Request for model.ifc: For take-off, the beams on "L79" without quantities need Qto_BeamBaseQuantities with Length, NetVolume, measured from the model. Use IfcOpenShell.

First a look at what the model holds.

```python
import ifcopenshell
import ifcopenshell.util.element
import ifcopenshell.util.unit

model = ifcopenshell.open("model.ifc")
print(model.schema)
for unit_type in ("LENGTHUNIT", "AREAUNIT", "VOLUMEUNIT"):
    print(unit_type, ifcopenshell.util.unit.calculate_unit_scale(model, unit_type))
storey = next(s for s in model.by_type("IfcBuildingStorey") if s.Name == "L79")
beams = [e for e in ifcopenshell.util.element.get_decomposition(storey) if e.is_a("IfcBeam")]
for e in sorted(beams, key=lambda e: e.id()):
    print(e.id(), e.is_a(), e.Name, list(ifcopenshell.util.element.get_psets(e, qtos_only=True)), sep=" | ")
```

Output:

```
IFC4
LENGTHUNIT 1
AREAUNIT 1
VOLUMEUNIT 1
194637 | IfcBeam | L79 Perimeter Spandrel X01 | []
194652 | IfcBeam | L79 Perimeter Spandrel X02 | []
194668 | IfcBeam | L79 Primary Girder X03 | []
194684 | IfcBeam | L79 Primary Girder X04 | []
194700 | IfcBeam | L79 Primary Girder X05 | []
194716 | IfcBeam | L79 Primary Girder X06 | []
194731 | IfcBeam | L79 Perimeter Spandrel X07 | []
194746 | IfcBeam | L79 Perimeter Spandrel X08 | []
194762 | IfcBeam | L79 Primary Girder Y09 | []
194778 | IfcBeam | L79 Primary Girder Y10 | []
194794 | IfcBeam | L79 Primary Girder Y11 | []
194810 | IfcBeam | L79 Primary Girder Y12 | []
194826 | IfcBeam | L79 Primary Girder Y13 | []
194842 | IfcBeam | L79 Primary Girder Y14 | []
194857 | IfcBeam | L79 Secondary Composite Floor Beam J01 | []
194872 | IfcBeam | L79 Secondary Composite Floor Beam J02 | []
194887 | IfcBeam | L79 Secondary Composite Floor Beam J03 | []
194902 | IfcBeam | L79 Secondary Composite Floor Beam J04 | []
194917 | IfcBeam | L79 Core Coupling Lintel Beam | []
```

```python
import ifcopenshell
import ifcopenshell.api.pset
import ifcopenshell.geom
import ifcopenshell.util.element
import ifcopenshell.util.shape
import ifcopenshell.util.unit

model = ifcopenshell.open("model.ifc")
unit_scale = ifcopenshell.util.unit.calculate_unit_scale(model)
volume_scale = ifcopenshell.util.unit.calculate_unit_scale(model, "VOLUMEUNIT")
settings = ifcopenshell.geom.settings()

storey = next(s for s in model.by_type("IfcBuildingStorey") if s.Name == "L79")
beams = [e for e in ifcopenshell.util.element.get_decomposition(storey) if e.is_a("IfcBeam")]

for e in sorted(beams, key=lambda e: e.id()):
    if ifcopenshell.util.element.get_psets(e, qtos_only=True, should_inherit=False):
        continue
    # Geometry comes back in metres, in the element's own axes.
    shape = ifcopenshell.geom.create_shape(settings, e)
    values = {
        "Length": ifcopenshell.util.shape.get_max_xyz(shape.geometry) / unit_scale,
        "NetVolume": ifcopenshell.util.shape.get_volume(shape.geometry) / volume_scale,
    }
    qto = ifcopenshell.api.pset.add_qto(model, product=e, name="Qto_BeamBaseQuantities")
    ifcopenshell.api.pset.edit_qto(model, qto=qto, properties=values)
    print(e.id(), {k: round(v, 3) for k, v in values.items()})

model.write("model_edited.ifc")
```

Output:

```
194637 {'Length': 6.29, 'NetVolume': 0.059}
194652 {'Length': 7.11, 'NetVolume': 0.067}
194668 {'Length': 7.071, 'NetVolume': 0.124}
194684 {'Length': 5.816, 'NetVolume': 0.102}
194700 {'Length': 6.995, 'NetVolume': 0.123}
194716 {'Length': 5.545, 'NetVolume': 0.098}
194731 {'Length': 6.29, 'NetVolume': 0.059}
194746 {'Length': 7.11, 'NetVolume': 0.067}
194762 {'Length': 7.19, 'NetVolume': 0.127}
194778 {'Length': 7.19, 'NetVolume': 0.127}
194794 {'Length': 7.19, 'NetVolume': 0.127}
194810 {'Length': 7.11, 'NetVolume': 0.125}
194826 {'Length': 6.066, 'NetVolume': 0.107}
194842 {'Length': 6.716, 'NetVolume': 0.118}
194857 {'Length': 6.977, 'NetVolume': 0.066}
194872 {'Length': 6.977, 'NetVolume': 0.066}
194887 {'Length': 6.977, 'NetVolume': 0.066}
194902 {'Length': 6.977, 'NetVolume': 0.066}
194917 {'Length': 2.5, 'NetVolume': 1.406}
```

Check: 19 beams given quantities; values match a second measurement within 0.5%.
